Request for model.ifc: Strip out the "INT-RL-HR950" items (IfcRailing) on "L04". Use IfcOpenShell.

First a look at what the model holds.

```python
import ifcopenshell
import ifcopenshell.util.element

model = ifcopenshell.open("model.ifc")
print(model.schema)
storey = next(s for s in model.by_type("IfcBuildingStorey") if s.Name == "L04")
railings = [e for e in ifcopenshell.util.element.get_decomposition(storey) if e.is_a("IfcRailing")]
seen = {}
for e in railings:
    element_type = ifcopenshell.util.element.get_type(e)
    name = element_type.Name if element_type not in (None, e) else None
    seen[name] = seen.get(name, 0) + 1
for name, count in sorted(seen.items(), key=str):
    print(count, "x", name)
```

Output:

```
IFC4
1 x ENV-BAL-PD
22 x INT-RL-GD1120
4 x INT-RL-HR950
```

```python
import ifcopenshell
import ifcopenshell.api.root
import ifcopenshell.util.element

model = ifcopenshell.open("model.ifc")

storey = next(s for s in model.by_type("IfcBuildingStorey") if s.Name == "L04")
railings = [e for e in ifcopenshell.util.element.get_decomposition(storey) if e.is_a("IfcRailing")]
targets = [e for e in railings if (t := ifcopenshell.util.element.get_type(e)) not in (None, e) and t.Name == "INT-RL-HR950"]

for e in targets:
    ifcopenshell.api.root.remove_product(model, product=e)
print(len(targets), "removed")

model.write("model_edited.ifc")
```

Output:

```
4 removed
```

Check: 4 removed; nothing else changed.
